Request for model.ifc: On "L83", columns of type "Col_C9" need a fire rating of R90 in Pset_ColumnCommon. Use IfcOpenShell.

First a look at what the model holds.

```python
import ifcopenshell
import ifcopenshell.util.element

model = ifcopenshell.open("model.ifc")
print(model.schema)
storey = next(s for s in model.by_type("IfcBuildingStorey") if s.Name == "L83")
columns = [e for e in ifcopenshell.util.element.get_decomposition(storey) if e.is_a("IfcColumn")]
seen = {}
for e in columns:
    element_type = ifcopenshell.util.element.get_type(e)
    key = (element_type.Name if element_type != e and element_type else None, ifcopenshell.util.element.get_pset(e, "Pset_ColumnCommon", "FireRating"))
    seen[key] = seen.get(key, 0) + 1
for (name, value), count in sorted(seen.items(), key=str):
    print(count, "x", name, "|", value)
```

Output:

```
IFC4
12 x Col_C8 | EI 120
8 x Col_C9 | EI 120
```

```python
import ifcopenshell
import ifcopenshell.api.pset
import ifcopenshell.util.element

model = ifcopenshell.open("model.ifc")

storey = next(s for s in model.by_type("IfcBuildingStorey") if s.Name == "L83")
columns = [e for e in ifcopenshell.util.element.get_decomposition(storey) if e.is_a("IfcColumn")]

count = 0
for e in columns:
    element_type = ifcopenshell.util.element.get_type(e)
    if element_type in (None, e) or element_type.Name != "Col_C9":
        continue
    found = ifcopenshell.util.element.get_pset(e, "Pset_ColumnCommon", should_inherit=False)
    if found:
        pset = model.by_id(found["id"])
        if len(ifcopenshell.util.element.get_elements_by_pset(pset)) > 1:
            pset = ifcopenshell.api.pset.unshare_pset(model, products=[e], pset=pset)[0]
    else:
        pset = ifcopenshell.api.pset.add_pset(model, product=e, name="Pset_ColumnCommon")
    ifcopenshell.api.pset.edit_pset(model, pset=pset, properties={"FireRating": "R90"})
    count += 1

print(count, "columns updated")

model.write("model_v2.ifc")
```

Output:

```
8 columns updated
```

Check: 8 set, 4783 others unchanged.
